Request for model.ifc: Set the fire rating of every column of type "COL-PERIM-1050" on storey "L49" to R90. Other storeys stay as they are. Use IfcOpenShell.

First a look at what the model holds.

```python
import ifcopenshell
import ifcopenshell.util.element

model = ifcopenshell.open("model.ifc")
print(model.schema)
storey = next(s for s in model.by_type("IfcBuildingStorey") if s.Name == "L49")
columns = [e for e in ifcopenshell.util.element.get_decomposition(storey) if e.is_a("IfcColumn")]
seen = {}
for e in columns:
    element_type = ifcopenshell.util.element.get_type(e)
    key = (element_type.Name if element_type != e and element_type else None, ifcopenshell.util.element.get_pset(e, "Pset_ColumnCommon", "FireRating"))
    seen[key] = seen.get(key, 0) + 1
for (name, value), count in sorted(seen.items(), key=str):
    print(count, "x", name, "|", value)
```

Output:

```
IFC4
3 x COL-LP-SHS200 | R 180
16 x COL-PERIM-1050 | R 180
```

```python
import ifcopenshell
import ifcopenshell.api.pset
import ifcopenshell.util.element

model = ifcopenshell.open("model.ifc")

storey = next(s for s in model.by_type("IfcBuildingStorey") if s.Name == "L49")
columns = [e for e in ifcopenshell.util.element.get_decomposition(storey) if e.is_a("IfcColumn")]

count = 0
for e in columns:
    element_type = ifcopenshell.util.element.get_type(e)
    if element_type in (None, e) or element_type.Name != "COL-PERIM-1050":
        continue
    found = ifcopenshell.util.element.get_pset(e, "Pset_ColumnCommon", should_inherit=False)
    if found:
        pset = model.by_id(found["id"])
        if len(ifcopenshell.util.element.get_elements_by_pset(pset)) > 1:
            pset = ifcopenshell.api.pset.unshare_pset(model, products=[e], pset=pset)[0]
    else:
        pset = ifcopenshell.api.pset.add_pset(model, product=e, name="Pset_ColumnCommon")
    ifcopenshell.api.pset.edit_pset(model, pset=pset, properties={"FireRating": "R90"})
    count += 1

print(count, "columns updated")

model.write("model_edited.ifc")
```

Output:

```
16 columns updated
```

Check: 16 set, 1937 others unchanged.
